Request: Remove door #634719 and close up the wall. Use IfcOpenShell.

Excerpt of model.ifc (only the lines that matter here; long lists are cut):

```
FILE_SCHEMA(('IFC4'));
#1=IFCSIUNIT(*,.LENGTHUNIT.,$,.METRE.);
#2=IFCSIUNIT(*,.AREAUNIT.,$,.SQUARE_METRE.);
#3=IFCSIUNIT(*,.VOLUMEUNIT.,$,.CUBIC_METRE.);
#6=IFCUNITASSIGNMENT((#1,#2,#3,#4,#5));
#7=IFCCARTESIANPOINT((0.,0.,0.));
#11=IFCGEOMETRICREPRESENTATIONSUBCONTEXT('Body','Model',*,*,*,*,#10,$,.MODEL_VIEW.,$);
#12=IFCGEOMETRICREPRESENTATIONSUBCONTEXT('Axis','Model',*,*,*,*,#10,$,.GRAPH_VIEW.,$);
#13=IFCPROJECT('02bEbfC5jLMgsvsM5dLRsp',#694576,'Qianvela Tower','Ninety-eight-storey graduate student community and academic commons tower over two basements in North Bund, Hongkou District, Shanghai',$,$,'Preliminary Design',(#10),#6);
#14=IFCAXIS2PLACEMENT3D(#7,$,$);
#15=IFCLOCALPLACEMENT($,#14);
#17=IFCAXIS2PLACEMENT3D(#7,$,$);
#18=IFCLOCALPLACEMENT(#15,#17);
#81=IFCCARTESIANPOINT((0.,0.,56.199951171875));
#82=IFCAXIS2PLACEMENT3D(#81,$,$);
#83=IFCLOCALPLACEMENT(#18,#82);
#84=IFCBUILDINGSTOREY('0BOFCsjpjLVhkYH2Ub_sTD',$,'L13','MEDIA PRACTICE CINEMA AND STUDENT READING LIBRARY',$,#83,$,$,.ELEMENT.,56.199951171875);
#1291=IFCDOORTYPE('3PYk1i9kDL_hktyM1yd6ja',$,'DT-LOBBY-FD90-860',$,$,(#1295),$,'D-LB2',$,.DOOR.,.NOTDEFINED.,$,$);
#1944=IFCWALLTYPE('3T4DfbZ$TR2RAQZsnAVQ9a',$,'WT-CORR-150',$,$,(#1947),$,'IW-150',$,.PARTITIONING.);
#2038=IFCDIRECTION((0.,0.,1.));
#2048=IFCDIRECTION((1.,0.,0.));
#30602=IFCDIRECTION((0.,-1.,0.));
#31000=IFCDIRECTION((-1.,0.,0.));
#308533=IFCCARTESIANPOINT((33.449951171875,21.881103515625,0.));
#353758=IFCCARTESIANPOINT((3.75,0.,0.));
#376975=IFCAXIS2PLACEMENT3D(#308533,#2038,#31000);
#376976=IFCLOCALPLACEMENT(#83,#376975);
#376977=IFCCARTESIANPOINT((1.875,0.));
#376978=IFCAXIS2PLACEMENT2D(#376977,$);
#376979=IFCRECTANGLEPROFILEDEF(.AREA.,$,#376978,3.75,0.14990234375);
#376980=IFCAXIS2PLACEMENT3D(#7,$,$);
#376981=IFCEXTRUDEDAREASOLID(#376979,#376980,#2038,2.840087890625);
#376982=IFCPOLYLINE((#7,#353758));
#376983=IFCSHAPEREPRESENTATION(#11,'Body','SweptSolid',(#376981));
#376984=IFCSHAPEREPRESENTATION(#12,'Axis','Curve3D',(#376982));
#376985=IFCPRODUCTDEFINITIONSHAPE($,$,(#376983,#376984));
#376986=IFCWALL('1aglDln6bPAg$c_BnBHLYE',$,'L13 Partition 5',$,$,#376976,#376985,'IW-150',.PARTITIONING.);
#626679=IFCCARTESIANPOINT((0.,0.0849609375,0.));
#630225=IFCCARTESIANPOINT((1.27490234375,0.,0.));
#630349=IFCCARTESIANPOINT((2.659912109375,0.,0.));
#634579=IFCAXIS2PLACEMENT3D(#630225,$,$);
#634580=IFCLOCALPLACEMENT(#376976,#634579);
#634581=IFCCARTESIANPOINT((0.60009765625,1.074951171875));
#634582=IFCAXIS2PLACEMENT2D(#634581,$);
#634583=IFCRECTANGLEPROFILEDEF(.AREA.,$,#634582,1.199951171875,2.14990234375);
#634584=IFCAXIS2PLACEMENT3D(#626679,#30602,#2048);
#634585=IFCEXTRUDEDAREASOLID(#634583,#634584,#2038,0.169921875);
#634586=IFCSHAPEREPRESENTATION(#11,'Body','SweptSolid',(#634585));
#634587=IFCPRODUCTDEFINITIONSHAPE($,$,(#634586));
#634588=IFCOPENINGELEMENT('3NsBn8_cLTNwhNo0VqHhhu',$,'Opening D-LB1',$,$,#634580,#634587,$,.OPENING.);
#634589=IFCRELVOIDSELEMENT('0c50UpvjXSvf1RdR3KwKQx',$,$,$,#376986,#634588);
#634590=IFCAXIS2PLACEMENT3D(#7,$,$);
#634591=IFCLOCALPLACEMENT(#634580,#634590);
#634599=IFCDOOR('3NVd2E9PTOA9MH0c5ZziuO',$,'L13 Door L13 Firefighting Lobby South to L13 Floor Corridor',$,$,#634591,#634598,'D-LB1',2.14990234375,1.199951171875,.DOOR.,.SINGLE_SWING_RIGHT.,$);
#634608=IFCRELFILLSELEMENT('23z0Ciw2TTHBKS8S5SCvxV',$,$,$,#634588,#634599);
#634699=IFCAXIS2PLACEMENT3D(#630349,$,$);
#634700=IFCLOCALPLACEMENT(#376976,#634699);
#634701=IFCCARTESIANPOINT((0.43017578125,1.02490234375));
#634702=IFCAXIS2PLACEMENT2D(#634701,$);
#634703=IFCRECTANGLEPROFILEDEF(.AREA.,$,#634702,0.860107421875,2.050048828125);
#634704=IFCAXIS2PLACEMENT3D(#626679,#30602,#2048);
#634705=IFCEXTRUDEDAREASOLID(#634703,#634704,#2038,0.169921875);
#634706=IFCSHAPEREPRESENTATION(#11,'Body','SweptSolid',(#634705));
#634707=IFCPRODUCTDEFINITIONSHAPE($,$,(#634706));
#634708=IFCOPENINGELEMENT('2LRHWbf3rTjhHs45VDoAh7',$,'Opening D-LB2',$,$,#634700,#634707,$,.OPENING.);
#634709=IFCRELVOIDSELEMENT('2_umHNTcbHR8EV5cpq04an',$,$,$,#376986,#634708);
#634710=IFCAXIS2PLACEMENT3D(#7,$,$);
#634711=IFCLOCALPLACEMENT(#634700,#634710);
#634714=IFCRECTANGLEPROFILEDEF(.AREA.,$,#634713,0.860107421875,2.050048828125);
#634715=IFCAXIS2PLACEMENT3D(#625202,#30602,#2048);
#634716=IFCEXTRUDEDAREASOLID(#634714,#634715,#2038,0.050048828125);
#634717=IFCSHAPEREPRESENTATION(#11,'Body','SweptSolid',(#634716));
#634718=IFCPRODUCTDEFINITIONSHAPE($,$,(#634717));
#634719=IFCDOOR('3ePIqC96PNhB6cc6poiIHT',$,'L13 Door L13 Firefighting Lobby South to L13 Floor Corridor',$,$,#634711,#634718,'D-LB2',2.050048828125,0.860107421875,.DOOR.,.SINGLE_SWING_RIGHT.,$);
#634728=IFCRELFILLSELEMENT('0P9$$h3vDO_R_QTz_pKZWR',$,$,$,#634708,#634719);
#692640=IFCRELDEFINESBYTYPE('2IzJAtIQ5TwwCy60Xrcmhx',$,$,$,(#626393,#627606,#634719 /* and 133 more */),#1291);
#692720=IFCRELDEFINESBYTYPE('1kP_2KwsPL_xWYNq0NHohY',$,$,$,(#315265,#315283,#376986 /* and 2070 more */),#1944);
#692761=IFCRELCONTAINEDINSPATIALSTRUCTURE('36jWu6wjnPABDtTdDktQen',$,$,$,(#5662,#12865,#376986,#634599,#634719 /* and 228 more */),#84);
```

```python
import ifcopenshell
import ifcopenshell.api.feature
import ifcopenshell.api.root
import ifcopenshell.geom
import ifcopenshell.util.shape

model = ifcopenshell.open("model.ifc")
settings = ifcopenshell.geom.settings()


def volume(element):
    """Net volume in cubic metres, openings subtracted."""
    shape = ifcopenshell.geom.create_shape(settings, element)
    return ifcopenshell.util.shape.get_volume(shape.geometry)


door = model.by_id(634719)
opening = door.FillsVoids[0].RelatingOpeningElement
wall = opening.VoidsElements[0].RelatingBuildingElement
before = volume(wall)

ifcopenshell.api.root.remove_product(model, product=door)
ifcopenshell.api.feature.remove_feature(model, feature=opening)

after = volume(wall)

print(f"wall volume {before:.3f} -> {after:.3f} m3")

model.write("model_edited.ifc")
```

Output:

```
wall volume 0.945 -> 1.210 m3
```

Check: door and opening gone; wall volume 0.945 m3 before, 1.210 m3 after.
